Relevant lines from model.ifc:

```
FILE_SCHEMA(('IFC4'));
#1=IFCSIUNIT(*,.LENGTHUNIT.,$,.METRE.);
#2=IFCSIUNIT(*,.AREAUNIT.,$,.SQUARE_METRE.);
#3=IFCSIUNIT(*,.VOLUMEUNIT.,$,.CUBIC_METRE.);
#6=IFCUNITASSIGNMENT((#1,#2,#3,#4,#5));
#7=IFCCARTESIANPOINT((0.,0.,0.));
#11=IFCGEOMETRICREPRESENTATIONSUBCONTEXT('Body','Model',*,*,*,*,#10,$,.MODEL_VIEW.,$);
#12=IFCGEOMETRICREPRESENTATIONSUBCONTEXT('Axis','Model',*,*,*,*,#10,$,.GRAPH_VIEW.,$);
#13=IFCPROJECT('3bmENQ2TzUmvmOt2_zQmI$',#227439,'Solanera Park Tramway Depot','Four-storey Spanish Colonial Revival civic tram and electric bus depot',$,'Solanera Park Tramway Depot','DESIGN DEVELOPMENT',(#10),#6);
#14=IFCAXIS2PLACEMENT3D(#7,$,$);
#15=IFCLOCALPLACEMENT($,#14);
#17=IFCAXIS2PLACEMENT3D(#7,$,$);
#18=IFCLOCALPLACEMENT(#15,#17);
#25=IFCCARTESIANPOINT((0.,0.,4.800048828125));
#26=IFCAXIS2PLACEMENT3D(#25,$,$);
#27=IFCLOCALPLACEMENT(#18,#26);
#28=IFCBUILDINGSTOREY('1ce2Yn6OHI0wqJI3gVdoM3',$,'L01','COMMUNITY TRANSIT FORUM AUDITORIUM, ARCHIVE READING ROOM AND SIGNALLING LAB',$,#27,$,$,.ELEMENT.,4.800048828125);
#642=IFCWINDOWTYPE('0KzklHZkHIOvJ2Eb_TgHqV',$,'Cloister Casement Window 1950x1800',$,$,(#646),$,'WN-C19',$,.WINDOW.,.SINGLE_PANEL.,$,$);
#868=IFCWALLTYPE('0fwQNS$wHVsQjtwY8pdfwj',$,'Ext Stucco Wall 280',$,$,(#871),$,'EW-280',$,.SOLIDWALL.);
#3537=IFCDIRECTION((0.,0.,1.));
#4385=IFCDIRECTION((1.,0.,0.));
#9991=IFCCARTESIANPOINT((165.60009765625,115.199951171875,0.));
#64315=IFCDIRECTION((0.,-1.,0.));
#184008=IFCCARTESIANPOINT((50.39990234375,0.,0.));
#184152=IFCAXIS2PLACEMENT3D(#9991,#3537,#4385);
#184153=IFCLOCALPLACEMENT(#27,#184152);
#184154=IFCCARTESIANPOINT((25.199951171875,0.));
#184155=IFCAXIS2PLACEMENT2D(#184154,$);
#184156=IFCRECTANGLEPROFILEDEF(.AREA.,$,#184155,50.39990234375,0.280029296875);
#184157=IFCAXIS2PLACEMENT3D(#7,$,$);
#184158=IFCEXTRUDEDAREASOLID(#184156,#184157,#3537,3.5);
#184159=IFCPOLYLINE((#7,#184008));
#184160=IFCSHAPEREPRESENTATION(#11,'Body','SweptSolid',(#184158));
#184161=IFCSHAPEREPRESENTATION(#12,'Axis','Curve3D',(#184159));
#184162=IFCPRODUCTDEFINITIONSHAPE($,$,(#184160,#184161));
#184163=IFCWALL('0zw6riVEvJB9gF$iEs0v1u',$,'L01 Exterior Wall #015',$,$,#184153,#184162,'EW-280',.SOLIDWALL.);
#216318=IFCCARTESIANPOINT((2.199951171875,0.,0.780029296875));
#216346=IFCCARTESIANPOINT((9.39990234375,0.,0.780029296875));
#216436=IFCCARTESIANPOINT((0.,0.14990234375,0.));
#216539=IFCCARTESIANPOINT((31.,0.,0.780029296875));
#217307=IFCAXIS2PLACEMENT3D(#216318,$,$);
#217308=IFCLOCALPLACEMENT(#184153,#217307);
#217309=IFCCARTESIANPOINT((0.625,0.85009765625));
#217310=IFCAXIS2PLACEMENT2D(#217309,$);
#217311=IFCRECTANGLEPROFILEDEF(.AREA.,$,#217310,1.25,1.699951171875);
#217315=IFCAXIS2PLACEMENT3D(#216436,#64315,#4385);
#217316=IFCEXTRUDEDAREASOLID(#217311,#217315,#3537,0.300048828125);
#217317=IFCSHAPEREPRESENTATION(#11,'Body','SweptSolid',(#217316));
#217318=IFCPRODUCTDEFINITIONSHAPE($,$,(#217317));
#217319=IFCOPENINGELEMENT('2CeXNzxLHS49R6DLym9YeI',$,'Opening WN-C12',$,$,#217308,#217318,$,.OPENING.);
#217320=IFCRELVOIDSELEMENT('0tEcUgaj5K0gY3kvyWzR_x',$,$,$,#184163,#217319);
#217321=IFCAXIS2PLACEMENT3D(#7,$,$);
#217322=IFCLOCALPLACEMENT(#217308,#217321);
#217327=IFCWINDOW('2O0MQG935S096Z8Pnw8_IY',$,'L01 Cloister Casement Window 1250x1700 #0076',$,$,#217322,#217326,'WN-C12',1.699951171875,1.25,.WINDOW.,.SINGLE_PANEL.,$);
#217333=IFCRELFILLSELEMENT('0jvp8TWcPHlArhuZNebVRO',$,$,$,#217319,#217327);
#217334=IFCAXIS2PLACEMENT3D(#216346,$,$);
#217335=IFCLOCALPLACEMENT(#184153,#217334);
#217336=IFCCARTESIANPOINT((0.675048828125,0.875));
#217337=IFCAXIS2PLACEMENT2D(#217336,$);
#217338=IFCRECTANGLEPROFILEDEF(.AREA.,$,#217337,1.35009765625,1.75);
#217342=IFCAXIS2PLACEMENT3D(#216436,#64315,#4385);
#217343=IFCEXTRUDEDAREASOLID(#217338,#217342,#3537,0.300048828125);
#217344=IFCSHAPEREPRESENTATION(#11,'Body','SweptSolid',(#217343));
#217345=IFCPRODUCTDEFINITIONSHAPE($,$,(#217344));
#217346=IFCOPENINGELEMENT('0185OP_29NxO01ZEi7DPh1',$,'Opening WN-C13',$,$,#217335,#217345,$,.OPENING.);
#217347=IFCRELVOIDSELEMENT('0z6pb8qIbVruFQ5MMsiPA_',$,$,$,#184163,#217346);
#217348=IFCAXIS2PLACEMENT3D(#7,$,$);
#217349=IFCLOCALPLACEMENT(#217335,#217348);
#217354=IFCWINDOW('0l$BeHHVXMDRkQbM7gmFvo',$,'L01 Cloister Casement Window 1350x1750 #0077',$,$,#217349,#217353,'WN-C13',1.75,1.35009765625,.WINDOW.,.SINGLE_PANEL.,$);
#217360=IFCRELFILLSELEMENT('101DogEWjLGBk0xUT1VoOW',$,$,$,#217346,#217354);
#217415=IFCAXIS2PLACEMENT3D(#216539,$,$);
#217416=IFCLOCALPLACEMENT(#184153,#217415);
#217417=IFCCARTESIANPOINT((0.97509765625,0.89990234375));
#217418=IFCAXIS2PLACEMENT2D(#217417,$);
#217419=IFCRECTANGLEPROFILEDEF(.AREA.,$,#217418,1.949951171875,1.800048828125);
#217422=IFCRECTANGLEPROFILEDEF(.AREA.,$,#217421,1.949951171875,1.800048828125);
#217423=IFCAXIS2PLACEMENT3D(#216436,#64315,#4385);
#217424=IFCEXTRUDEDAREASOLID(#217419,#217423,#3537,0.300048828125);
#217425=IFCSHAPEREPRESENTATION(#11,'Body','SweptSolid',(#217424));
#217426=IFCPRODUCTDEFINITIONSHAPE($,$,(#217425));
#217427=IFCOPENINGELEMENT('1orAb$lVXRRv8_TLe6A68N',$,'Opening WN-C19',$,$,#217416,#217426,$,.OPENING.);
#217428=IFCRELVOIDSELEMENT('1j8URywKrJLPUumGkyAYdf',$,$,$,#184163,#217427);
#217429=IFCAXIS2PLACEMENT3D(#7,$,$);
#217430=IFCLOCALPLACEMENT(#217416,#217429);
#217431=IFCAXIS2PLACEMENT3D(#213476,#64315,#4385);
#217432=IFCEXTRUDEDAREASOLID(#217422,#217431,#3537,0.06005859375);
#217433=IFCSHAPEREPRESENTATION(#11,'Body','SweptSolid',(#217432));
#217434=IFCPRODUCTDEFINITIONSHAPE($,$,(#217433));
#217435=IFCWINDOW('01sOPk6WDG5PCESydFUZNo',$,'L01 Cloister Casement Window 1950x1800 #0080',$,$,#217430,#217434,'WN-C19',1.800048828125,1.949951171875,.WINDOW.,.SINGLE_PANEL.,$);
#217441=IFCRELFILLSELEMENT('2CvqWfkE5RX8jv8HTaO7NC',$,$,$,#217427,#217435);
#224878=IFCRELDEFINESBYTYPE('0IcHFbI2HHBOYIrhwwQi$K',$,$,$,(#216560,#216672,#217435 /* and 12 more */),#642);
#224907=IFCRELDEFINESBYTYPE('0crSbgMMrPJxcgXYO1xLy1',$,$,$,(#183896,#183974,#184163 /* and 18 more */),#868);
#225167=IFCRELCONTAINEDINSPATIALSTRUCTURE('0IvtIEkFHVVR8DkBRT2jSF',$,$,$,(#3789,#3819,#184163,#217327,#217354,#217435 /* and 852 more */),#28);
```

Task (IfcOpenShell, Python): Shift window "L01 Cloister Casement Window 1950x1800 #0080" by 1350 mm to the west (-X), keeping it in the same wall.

```python
import ifcopenshell
import ifcopenshell.api.geometry
import ifcopenshell.util.placement
import ifcopenshell.util.unit

model = ifcopenshell.open("model.ifc")
unit_scale = ifcopenshell.util.unit.calculate_unit_scale(model)

window = model.by_guid("01sOPk6WDG5PCESydFUZNo")
opening = window.FillsVoids[0].RelatingOpeningElement
wall = opening.VoidsElements[0].RelatingBuildingElement

wall_matrix = ifcopenshell.util.placement.get_local_placement(wall.ObjectPlacement)
shift = wall_matrix[:3, 0] * -1.35 / unit_scale
before = ifcopenshell.util.placement.get_local_placement(window.ObjectPlacement)[:3, 3].copy()

# The window is placed relative to its opening, so it follows when the opening moves.
matrix = ifcopenshell.util.placement.get_local_placement(opening.ObjectPlacement)
matrix[:3, 3] += shift
ifcopenshell.api.geometry.edit_object_placement(
    model, product=opening, matrix=matrix, is_si=False, should_transform_children=True
)

after = ifcopenshell.util.placement.get_local_placement(window.ObjectPlacement)[:3, 3]
print("window moved by", (after - before).round(3) + 0.0)

model.write("model_edited.ifc")
```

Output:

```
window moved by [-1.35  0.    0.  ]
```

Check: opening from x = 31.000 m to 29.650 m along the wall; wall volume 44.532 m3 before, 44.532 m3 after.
